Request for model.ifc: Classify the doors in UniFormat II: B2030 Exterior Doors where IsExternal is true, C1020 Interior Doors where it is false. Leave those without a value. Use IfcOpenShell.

First a look at what the model holds.

```python
import ifcopenshell
import ifcopenshell.util.element

model = ifcopenshell.open("model.ifc")
print(model.schema)
print("classifications:", [c.Name for c in model.by_type("IfcClassification")])
values = [ifcopenshell.util.element.get_pset(e, "Pset_DoorCommon", "IsExternal") for e in model.by_type("IfcDoor")]
for value in (True, False, None):
    print("IsExternal", value, values.count(value))
```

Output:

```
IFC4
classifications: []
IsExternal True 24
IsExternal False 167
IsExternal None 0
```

```python
import ifcopenshell
import ifcopenshell.api.classification
import ifcopenshell.util.element

model = ifcopenshell.open("model.ifc")

system = ifcopenshell.api.classification.add_classification(model, classification="UniFormat II")

doors = model.by_type("IfcDoor")
external = {e: ifcopenshell.util.element.get_pset(e, "Pset_DoorCommon", "IsExternal") for e in doors}
for flag, code, name in ((True, "B2030", "Exterior Doors"), (False, "C1020", "Interior Doors")):
    products = [e for e in doors if external[e] is flag]
    ifcopenshell.api.classification.add_reference(
        model, products=products, classification=system, identification=code, name=name
    )
    print(code, len(products))

model.write("model_v2.ifc")
```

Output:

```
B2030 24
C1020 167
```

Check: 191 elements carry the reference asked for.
